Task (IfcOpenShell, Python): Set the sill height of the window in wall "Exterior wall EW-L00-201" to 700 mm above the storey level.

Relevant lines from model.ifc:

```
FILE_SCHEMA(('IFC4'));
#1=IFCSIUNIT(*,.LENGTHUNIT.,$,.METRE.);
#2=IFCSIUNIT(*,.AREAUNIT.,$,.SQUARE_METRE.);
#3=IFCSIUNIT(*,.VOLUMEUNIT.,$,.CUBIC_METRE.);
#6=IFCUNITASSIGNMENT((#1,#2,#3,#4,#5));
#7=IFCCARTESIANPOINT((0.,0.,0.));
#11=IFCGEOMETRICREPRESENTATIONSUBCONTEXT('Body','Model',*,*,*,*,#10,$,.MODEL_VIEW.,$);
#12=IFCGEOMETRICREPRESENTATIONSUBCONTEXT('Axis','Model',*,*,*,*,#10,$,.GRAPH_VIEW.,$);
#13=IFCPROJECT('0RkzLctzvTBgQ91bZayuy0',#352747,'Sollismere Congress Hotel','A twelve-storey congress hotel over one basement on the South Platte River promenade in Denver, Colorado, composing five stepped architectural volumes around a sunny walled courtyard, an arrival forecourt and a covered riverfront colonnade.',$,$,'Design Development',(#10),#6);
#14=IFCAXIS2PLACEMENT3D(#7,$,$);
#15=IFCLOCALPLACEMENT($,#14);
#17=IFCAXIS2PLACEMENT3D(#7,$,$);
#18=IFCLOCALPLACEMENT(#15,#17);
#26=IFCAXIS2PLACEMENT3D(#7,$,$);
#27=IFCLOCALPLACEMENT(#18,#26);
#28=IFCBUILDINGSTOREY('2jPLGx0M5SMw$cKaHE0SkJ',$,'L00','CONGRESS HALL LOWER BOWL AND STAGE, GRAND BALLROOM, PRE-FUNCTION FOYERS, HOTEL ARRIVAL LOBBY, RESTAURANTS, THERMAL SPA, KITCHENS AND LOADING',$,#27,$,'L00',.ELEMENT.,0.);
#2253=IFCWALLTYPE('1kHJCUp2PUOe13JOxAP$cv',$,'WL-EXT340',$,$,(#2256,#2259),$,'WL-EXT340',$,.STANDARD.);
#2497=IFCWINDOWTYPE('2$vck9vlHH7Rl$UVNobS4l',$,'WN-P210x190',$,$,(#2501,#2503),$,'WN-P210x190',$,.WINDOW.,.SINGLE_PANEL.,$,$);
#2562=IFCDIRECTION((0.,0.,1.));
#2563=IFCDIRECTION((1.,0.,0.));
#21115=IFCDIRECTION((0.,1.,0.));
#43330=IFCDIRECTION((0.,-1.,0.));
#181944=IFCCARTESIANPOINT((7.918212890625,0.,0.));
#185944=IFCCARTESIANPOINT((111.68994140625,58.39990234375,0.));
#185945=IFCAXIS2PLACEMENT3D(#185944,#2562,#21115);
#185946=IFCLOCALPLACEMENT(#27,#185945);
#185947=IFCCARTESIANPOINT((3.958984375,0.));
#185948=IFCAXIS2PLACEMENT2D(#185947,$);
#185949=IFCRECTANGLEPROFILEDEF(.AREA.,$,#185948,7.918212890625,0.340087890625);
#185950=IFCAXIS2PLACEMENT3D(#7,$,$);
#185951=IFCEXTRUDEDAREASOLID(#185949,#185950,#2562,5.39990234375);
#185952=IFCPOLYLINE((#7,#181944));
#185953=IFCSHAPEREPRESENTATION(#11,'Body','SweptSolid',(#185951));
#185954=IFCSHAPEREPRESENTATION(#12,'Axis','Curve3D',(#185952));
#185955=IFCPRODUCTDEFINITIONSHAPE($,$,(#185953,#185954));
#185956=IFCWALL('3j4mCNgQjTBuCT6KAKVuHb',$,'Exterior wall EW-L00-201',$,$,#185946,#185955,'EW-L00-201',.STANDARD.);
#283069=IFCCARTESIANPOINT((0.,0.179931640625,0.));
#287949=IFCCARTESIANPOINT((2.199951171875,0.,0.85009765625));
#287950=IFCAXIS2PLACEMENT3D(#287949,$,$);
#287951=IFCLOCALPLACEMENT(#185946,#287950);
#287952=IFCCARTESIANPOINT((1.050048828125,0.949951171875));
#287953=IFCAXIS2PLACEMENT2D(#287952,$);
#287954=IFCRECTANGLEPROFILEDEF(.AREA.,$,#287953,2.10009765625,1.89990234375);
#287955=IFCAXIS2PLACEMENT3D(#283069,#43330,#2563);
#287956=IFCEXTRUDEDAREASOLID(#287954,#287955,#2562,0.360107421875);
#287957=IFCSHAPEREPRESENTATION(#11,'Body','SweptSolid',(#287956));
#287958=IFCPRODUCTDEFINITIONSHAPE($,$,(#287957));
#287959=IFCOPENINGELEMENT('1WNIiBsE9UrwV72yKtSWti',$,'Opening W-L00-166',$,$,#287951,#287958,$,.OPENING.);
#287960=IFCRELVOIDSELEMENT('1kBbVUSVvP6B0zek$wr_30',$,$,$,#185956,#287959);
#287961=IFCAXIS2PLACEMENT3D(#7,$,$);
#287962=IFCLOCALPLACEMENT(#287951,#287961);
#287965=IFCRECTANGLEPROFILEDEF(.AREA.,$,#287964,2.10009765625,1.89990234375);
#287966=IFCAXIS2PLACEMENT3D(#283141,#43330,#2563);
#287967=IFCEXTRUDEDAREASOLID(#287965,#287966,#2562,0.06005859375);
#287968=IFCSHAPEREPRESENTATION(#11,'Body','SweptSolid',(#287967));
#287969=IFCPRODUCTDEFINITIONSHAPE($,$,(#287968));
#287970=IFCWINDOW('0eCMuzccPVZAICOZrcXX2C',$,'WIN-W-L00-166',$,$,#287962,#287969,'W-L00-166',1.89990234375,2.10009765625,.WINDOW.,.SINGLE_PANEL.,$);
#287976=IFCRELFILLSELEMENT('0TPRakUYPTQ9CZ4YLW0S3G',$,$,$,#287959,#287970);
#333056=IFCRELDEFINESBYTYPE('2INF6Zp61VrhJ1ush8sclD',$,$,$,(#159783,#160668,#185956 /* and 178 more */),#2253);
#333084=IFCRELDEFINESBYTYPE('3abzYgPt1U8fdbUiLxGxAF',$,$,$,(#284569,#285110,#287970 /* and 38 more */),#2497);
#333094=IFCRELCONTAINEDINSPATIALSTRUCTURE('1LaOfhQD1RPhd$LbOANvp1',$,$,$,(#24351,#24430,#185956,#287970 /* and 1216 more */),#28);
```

```python
import numpy as np
import ifcopenshell
import ifcopenshell.api.geometry
import ifcopenshell.geom
import ifcopenshell.util.element
import ifcopenshell.util.placement
import ifcopenshell.util.shape
import ifcopenshell.util.unit

model = ifcopenshell.open("model.ifc")
unit_scale = ifcopenshell.util.unit.calculate_unit_scale(model)

window = model.by_guid("0eCMuzccPVZAICOZrcXX2C")
opening = window.FillsVoids[0].RelatingOpeningElement
storey = ifcopenshell.util.element.get_container(window, ifc_class="IfcBuildingStorey")
level = ifcopenshell.util.placement.get_local_placement(storey.ObjectPlacement)[2, 3]

# The opening's origin need not be at the sill, so measure its lowest point.
shape = ifcopenshell.geom.create_shape(ifcopenshell.geom.settings(), opening)
bottom = ifcopenshell.util.shape.get_shape_bottom_elevation(shape, shape.geometry) / unit_scale
dz = level + 0.7 / unit_scale - bottom

shift = np.array([0.0, 0.0, dz])
# The window is placed relative to its opening, so it follows when the opening moves.
matrix = ifcopenshell.util.placement.get_local_placement(opening.ObjectPlacement)
matrix[:3, 3] += shift
ifcopenshell.api.geometry.edit_object_placement(
    model, product=opening, matrix=matrix, is_si=False, should_transform_children=True
)

print(f"moved by {dz * unit_scale:+.3f} m")

model.write("model_v2.ifc")
```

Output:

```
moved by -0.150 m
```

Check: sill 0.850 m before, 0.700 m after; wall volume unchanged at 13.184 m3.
